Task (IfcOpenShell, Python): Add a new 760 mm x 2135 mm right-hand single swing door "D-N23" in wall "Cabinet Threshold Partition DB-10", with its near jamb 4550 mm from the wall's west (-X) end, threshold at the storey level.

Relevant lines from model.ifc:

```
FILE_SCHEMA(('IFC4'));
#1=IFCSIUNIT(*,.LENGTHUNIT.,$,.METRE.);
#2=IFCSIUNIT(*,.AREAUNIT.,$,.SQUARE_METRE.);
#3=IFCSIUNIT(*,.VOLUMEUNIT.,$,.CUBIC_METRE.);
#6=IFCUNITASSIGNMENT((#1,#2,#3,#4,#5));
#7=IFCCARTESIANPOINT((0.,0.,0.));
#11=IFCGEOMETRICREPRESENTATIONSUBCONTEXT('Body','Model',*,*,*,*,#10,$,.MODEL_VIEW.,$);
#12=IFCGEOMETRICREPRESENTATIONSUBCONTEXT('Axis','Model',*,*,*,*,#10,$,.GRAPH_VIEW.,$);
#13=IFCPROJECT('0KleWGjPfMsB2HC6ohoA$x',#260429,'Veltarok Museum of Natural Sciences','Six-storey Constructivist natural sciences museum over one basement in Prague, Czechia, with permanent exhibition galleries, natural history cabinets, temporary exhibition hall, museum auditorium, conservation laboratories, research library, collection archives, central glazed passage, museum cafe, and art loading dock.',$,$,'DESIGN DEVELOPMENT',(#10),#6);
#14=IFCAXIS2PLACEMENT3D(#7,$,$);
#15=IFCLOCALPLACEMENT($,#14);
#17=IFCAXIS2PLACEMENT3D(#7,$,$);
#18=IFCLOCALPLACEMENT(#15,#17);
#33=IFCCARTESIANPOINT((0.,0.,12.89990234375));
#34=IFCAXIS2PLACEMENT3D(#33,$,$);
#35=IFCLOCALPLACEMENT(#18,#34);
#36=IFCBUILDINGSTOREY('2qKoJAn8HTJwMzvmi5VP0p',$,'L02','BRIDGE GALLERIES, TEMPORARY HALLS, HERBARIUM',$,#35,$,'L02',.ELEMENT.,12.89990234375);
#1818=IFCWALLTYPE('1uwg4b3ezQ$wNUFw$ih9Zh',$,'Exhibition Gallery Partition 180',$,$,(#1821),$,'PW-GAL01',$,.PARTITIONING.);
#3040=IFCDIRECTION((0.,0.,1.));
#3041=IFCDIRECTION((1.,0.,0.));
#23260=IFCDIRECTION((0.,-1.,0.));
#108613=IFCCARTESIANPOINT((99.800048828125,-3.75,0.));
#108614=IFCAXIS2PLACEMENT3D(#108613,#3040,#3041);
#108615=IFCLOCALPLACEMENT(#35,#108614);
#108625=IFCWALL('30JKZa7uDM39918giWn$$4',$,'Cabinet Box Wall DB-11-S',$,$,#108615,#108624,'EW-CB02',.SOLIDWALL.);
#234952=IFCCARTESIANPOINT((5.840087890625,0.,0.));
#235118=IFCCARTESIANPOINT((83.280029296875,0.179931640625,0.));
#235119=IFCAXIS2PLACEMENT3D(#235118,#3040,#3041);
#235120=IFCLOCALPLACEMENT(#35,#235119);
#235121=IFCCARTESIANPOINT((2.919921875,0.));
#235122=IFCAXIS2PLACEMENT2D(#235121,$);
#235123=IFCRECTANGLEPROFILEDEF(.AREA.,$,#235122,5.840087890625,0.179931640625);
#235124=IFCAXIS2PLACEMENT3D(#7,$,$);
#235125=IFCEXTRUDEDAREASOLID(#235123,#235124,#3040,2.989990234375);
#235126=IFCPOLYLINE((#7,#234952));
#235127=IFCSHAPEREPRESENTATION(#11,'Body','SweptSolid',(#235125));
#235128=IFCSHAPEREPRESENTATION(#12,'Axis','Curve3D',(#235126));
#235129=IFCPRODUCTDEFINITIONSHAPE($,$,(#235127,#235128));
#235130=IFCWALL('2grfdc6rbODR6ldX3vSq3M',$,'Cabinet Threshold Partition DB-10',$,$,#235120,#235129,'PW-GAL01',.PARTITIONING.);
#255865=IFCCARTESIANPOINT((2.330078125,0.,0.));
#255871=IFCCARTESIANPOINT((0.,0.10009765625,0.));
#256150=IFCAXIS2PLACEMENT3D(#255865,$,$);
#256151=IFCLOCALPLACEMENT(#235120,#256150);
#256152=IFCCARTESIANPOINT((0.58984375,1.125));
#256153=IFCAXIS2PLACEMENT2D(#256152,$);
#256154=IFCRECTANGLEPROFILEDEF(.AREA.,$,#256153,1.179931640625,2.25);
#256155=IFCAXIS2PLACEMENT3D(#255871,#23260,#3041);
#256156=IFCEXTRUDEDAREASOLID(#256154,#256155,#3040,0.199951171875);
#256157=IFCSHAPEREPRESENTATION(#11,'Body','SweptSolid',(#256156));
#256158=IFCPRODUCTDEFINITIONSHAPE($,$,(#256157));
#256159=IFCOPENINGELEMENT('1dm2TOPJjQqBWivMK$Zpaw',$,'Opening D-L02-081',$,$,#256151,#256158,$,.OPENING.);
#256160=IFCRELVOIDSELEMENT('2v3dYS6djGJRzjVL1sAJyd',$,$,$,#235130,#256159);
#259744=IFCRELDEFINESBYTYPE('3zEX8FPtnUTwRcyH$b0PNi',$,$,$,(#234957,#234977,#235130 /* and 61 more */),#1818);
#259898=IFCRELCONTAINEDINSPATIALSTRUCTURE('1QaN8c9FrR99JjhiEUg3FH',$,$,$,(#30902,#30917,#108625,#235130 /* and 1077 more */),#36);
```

```python
import numpy as np
import ifcopenshell
import ifcopenshell.api.feature
import ifcopenshell.api.geometry
import ifcopenshell.api.root
import ifcopenshell.api.spatial
import ifcopenshell.geom
import ifcopenshell.util.element
import ifcopenshell.util.placement
import ifcopenshell.util.representation
import ifcopenshell.util.shape
import ifcopenshell.util.unit

model = ifcopenshell.open("model.ifc")
unit_scale = ifcopenshell.util.unit.calculate_unit_scale(model)
settings = ifcopenshell.geom.settings()


def volume(element):
    """Net volume in cubic metres, openings subtracted."""
    shape = ifcopenshell.geom.create_shape(settings, element)
    return ifcopenshell.util.shape.get_volume(shape.geometry)


wall = model.by_id(235130)
storey = ifcopenshell.util.element.get_container(wall, ifc_class="IfcBuildingStorey")
context = ifcopenshell.util.representation.get_context(model, "Model", "Body", "MODEL_VIEW")
before = volume(wall)

width, height, from_end, sill = 0.76, 2.135, 4.55, 0.0  # metres

# The wall runs along its own X axis, and the end named is its -X end.
wall_shape = ifcopenshell.geom.create_shape(settings, wall)
x, y, z = ifcopenshell.util.shape.get_vertices(wall_shape.geometry).T
start = x.min() + from_end
face, thickness = float(y.min()), float(y.max() - y.min())
wall_matrix = ifcopenshell.util.placement.get_local_placement(wall.ObjectPlacement)
level = ifcopenshell.util.placement.get_local_placement(storey.ObjectPlacement)[2, 3]


def in_wall(x, y):
    """Placement at x, y metres in the wall's axes, at sill height."""
    matrix = wall_matrix.copy()
    matrix[:, 3] = wall_matrix @ np.array([x / unit_scale, y / unit_scale, 0.0, 1.0])
    matrix[2, 3] = level + sill / unit_scale
    return matrix


# Opening: a box that overshoots both wall faces by 50 mm.
opening = ifcopenshell.api.root.create_entity(model, ifc_class="IfcOpeningElement", predefined_type="OPENING")
box = ifcopenshell.api.geometry.add_wall_representation(
    model, context=context, length=width, height=height, thickness=thickness + 0.1
)
ifcopenshell.api.geometry.assign_representation(model, product=opening, representation=box)
ifcopenshell.api.geometry.edit_object_placement(model, product=opening, matrix=in_wall(start, face - 0.05), is_si=False)
ifcopenshell.api.feature.add_feature(model, feature=opening, element=wall)

door = ifcopenshell.api.root.create_entity(model, ifc_class="IfcDoor", name="D-N23", predefined_type="DOOR")
door.OverallWidth, door.OverallHeight = width / unit_scale, height / unit_scale
door.OperationType = "SINGLE_SWING_RIGHT"
body = ifcopenshell.api.geometry.add_door_representation(
    model,
    context=context,
    overall_width=door.OverallWidth,
    overall_height=door.OverallHeight,
    operation_type="SINGLE_SWING_RIGHT",
    lining_properties={"LiningDepth": thickness / unit_scale, "ThresholdDepth": thickness / unit_scale},
)
ifcopenshell.api.geometry.assign_representation(model, product=door, representation=body)
ifcopenshell.api.spatial.assign_container(model, products=[door], relating_structure=storey)
ifcopenshell.api.feature.add_filling(model, opening=opening, element=door)

# The lining spans the wall, so the door starts at the wall face.
ifcopenshell.api.geometry.edit_object_placement(model, product=door, matrix=in_wall(start, face), is_si=False)

after = volume(wall)

print(f"wall volume {before:.3f} -> {after:.3f} m3")

model.write("model_updated.ifc")
```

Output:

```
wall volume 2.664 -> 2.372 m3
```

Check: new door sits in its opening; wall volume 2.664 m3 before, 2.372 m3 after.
